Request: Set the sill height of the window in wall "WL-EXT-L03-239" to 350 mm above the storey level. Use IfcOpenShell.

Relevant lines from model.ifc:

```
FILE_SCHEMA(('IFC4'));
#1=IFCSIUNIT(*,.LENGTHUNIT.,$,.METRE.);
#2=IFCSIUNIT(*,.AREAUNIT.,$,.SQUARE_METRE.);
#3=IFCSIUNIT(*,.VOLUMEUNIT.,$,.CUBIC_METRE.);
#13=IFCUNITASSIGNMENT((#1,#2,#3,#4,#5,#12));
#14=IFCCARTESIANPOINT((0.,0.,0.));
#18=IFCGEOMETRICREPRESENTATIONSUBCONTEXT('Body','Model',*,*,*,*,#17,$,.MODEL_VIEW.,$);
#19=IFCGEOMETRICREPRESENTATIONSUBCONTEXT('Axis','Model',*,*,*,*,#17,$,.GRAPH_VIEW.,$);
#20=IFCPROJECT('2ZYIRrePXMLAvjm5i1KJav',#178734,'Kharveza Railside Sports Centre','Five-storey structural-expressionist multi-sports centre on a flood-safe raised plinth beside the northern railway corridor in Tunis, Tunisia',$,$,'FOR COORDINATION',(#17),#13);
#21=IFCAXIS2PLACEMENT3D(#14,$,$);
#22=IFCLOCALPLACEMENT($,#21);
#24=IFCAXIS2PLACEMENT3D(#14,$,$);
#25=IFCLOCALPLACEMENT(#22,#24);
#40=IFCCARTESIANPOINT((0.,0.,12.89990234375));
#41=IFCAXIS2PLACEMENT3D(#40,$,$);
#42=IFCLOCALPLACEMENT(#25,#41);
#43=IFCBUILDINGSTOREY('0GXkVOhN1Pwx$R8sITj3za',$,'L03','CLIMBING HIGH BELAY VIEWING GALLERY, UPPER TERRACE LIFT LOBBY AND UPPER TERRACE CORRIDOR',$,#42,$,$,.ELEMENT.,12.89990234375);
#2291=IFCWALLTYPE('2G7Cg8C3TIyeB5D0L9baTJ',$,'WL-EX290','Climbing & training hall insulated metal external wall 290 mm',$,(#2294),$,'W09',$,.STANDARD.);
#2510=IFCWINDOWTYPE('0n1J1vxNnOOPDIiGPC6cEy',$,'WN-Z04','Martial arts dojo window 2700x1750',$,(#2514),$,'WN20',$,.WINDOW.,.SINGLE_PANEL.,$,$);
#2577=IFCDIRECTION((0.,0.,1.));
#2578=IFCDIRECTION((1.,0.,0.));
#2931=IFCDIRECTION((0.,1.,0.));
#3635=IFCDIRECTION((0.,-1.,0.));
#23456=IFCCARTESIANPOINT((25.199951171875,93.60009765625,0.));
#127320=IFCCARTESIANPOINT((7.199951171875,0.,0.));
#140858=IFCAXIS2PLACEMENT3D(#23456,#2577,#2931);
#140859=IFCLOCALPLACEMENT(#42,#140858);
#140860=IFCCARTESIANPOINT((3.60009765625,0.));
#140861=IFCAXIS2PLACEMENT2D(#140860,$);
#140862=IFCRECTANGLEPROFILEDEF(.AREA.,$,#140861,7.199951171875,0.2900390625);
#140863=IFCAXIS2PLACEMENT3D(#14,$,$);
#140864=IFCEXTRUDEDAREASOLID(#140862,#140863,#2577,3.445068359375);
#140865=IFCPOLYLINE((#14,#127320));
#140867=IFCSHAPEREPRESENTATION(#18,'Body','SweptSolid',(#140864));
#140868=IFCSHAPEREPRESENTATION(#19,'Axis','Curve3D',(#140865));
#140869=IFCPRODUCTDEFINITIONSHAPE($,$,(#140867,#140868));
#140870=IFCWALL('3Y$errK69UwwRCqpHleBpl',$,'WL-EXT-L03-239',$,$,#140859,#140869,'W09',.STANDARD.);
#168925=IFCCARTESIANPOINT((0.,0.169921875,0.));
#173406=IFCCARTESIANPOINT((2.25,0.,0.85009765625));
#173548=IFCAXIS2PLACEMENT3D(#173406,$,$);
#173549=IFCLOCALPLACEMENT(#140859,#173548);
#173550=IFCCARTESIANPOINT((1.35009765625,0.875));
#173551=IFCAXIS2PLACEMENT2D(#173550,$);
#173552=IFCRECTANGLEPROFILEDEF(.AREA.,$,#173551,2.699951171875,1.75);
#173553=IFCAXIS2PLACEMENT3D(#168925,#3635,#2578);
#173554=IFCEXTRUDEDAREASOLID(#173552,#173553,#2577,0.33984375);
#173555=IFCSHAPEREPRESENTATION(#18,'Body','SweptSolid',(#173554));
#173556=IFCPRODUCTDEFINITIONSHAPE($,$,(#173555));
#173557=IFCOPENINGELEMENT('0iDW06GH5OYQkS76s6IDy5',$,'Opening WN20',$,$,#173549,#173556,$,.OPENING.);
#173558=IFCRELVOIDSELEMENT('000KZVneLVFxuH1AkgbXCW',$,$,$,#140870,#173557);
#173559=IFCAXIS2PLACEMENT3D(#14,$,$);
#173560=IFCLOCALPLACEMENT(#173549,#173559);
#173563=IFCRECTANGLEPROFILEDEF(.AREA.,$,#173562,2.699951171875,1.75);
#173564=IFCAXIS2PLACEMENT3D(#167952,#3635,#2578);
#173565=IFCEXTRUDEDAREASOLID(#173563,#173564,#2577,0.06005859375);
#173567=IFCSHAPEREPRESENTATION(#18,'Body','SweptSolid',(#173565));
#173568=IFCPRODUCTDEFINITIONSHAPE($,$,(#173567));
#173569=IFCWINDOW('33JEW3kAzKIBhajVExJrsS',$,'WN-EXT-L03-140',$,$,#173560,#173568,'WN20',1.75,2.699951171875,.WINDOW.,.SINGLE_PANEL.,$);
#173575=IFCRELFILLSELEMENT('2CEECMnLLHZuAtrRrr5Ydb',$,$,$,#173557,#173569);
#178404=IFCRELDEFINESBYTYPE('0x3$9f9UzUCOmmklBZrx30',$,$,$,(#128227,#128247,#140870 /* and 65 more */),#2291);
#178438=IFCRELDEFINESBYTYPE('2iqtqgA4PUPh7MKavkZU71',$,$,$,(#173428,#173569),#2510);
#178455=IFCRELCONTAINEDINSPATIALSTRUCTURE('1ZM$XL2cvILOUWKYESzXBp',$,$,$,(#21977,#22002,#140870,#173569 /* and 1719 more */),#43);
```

```python
import numpy as np
import ifcopenshell
import ifcopenshell.api.geometry
import ifcopenshell.geom
import ifcopenshell.util.element
import ifcopenshell.util.placement
import ifcopenshell.util.shape
import ifcopenshell.util.unit

model = ifcopenshell.open("model.ifc")
unit_scale = ifcopenshell.util.unit.calculate_unit_scale(model)

window = model.by_guid("33JEW3kAzKIBhajVExJrsS")
opening = window.FillsVoids[0].RelatingOpeningElement
storey = ifcopenshell.util.element.get_container(window, ifc_class="IfcBuildingStorey")
level = ifcopenshell.util.placement.get_local_placement(storey.ObjectPlacement)[2, 3]

# The opening's origin need not be at the sill, so measure its lowest point.
shape = ifcopenshell.geom.create_shape(ifcopenshell.geom.settings(), opening)
bottom = ifcopenshell.util.shape.get_shape_bottom_elevation(shape, shape.geometry) / unit_scale
dz = level + 0.35 / unit_scale - bottom

shift = np.array([0.0, 0.0, dz])
# The window is placed relative to its opening, so it follows when the opening moves.
matrix = ifcopenshell.util.placement.get_local_placement(opening.ObjectPlacement)
matrix[:3, 3] += shift
ifcopenshell.api.geometry.edit_object_placement(
    model, product=opening, matrix=matrix, is_si=False, should_transform_children=True
)

print(f"moved by {dz * unit_scale:+.3f} m")

model.write("model_v2.ifc")
```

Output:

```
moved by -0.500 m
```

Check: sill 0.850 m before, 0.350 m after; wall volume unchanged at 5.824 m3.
